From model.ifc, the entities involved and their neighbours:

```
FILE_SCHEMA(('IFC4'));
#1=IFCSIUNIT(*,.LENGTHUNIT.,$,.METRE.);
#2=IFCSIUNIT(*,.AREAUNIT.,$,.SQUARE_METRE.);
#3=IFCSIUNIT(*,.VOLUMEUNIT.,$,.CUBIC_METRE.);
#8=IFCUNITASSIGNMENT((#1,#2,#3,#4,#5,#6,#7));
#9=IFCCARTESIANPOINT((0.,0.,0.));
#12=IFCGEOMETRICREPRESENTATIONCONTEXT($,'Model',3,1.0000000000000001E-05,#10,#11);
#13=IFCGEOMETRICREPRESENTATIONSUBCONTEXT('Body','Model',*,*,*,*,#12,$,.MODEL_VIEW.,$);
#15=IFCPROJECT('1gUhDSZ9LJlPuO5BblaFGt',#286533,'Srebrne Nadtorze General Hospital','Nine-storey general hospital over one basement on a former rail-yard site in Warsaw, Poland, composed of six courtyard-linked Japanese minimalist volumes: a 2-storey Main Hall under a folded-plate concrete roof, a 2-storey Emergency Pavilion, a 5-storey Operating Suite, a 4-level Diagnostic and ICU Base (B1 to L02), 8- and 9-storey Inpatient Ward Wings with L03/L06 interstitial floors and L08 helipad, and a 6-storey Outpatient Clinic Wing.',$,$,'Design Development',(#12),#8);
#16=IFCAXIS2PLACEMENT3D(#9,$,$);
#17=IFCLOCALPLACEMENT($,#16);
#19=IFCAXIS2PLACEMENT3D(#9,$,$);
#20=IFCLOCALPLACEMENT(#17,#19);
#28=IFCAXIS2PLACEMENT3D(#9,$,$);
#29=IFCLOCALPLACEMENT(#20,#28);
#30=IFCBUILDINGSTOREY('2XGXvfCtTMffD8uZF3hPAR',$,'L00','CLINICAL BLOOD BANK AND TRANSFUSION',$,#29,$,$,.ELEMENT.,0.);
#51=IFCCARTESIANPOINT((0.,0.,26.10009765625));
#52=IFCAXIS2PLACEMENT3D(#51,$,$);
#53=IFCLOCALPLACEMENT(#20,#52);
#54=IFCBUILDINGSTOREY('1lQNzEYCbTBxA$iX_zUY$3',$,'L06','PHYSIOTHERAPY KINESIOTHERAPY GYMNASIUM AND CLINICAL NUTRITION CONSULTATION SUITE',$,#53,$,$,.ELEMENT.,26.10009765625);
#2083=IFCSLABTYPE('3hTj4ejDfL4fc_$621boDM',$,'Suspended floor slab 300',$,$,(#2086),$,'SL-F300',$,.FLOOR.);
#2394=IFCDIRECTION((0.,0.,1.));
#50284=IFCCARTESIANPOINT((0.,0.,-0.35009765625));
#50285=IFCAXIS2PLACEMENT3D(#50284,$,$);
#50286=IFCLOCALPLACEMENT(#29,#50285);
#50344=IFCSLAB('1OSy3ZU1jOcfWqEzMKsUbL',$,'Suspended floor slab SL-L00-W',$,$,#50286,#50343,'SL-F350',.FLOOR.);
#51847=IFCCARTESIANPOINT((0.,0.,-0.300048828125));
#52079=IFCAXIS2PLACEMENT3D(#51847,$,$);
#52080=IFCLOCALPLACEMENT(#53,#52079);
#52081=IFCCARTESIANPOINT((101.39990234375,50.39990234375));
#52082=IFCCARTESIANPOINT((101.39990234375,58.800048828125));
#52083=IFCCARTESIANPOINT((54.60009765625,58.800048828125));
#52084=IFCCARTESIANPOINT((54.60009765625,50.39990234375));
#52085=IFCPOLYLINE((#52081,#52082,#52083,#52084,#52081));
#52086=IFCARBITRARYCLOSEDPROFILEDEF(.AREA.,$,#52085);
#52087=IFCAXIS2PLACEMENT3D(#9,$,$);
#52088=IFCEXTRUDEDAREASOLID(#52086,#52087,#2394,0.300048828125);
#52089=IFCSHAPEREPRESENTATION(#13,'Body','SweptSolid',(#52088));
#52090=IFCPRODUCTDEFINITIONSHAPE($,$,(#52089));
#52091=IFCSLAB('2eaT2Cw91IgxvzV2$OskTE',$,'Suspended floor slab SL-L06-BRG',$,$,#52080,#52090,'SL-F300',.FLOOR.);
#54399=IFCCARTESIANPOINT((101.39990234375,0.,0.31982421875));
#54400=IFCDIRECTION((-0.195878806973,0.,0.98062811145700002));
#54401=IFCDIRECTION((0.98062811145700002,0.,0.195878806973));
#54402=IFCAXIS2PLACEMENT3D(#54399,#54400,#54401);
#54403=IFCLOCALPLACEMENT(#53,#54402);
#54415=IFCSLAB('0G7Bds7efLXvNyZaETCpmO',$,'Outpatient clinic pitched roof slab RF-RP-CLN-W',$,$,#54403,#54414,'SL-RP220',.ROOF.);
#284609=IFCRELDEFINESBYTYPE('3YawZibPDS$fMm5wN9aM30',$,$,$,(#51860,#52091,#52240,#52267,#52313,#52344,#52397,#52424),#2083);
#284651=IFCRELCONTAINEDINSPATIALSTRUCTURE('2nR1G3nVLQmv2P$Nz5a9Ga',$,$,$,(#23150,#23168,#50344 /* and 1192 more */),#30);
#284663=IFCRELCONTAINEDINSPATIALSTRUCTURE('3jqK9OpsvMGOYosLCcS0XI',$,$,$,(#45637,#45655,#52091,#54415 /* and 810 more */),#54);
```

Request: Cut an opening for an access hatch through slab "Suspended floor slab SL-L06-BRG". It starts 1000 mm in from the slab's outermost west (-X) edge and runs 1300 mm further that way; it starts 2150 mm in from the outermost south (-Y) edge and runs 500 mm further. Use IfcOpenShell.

```python
import numpy as np
import ifcopenshell
import ifcopenshell.api.feature
import ifcopenshell.api.geometry
import ifcopenshell.api.root
import ifcopenshell.geom
import ifcopenshell.util.placement
import ifcopenshell.util.representation
import ifcopenshell.util.shape
import ifcopenshell.util.unit

model = ifcopenshell.open("model.ifc")
unit_scale = ifcopenshell.util.unit.calculate_unit_scale(model)
settings = ifcopenshell.geom.settings()


def volume(element):
    """Net volume in cubic metres, openings subtracted."""
    shape = ifcopenshell.geom.create_shape(settings, element)
    return ifcopenshell.util.shape.get_volume(shape.geometry)


slab = model.by_guid("2eaT2Cw91IgxvzV2$OskTE")
before = volume(slab)

# Extent in the slab's own axes, in metres. The edges named are its -X and -Y sides.
slab_shape = ifcopenshell.geom.create_shape(settings, slab)
vertices = ifcopenshell.util.shape.get_vertices(slab_shape.geometry)
x_min, y_min, bottom = vertices.min(axis=0)
top = vertices[:, 2].max()

opening = ifcopenshell.api.root.create_entity(model, ifc_class="IfcOpeningElement", name="Access hatch opening", predefined_type="OPENING")
context = ifcopenshell.util.representation.get_context(model, "Model", "Body", "MODEL_VIEW")
width, depth = 1.3, 0.5
outline = [(0.0, 0.0), (width, 0.0), (width, depth), (0.0, depth), (0.0, 0.0)]
# Overshoot both faces by 50 mm so the cut is clean.
shape = ifcopenshell.api.geometry.add_slab_representation(
    model, context=context, depth=top - bottom + 0.1, polyline=outline
)
ifcopenshell.api.geometry.assign_representation(model, product=opening, representation=shape)

matrix = ifcopenshell.util.placement.get_local_placement(slab.ObjectPlacement)
matrix[:, 3] = matrix @ np.append(np.array([x_min + 1, y_min + 2.15, bottom - 0.05]) / unit_scale, 1.0)
ifcopenshell.api.geometry.edit_object_placement(model, product=opening, matrix=matrix, is_si=False)
ifcopenshell.api.feature.add_feature(model, feature=opening, element=slab)

after = volume(slab)

print(f"slab volume {before:.3f} -> {after:.3f} m3")

model.write("model_rev.ifc")
```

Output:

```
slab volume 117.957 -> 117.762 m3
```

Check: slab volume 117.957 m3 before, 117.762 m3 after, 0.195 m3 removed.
